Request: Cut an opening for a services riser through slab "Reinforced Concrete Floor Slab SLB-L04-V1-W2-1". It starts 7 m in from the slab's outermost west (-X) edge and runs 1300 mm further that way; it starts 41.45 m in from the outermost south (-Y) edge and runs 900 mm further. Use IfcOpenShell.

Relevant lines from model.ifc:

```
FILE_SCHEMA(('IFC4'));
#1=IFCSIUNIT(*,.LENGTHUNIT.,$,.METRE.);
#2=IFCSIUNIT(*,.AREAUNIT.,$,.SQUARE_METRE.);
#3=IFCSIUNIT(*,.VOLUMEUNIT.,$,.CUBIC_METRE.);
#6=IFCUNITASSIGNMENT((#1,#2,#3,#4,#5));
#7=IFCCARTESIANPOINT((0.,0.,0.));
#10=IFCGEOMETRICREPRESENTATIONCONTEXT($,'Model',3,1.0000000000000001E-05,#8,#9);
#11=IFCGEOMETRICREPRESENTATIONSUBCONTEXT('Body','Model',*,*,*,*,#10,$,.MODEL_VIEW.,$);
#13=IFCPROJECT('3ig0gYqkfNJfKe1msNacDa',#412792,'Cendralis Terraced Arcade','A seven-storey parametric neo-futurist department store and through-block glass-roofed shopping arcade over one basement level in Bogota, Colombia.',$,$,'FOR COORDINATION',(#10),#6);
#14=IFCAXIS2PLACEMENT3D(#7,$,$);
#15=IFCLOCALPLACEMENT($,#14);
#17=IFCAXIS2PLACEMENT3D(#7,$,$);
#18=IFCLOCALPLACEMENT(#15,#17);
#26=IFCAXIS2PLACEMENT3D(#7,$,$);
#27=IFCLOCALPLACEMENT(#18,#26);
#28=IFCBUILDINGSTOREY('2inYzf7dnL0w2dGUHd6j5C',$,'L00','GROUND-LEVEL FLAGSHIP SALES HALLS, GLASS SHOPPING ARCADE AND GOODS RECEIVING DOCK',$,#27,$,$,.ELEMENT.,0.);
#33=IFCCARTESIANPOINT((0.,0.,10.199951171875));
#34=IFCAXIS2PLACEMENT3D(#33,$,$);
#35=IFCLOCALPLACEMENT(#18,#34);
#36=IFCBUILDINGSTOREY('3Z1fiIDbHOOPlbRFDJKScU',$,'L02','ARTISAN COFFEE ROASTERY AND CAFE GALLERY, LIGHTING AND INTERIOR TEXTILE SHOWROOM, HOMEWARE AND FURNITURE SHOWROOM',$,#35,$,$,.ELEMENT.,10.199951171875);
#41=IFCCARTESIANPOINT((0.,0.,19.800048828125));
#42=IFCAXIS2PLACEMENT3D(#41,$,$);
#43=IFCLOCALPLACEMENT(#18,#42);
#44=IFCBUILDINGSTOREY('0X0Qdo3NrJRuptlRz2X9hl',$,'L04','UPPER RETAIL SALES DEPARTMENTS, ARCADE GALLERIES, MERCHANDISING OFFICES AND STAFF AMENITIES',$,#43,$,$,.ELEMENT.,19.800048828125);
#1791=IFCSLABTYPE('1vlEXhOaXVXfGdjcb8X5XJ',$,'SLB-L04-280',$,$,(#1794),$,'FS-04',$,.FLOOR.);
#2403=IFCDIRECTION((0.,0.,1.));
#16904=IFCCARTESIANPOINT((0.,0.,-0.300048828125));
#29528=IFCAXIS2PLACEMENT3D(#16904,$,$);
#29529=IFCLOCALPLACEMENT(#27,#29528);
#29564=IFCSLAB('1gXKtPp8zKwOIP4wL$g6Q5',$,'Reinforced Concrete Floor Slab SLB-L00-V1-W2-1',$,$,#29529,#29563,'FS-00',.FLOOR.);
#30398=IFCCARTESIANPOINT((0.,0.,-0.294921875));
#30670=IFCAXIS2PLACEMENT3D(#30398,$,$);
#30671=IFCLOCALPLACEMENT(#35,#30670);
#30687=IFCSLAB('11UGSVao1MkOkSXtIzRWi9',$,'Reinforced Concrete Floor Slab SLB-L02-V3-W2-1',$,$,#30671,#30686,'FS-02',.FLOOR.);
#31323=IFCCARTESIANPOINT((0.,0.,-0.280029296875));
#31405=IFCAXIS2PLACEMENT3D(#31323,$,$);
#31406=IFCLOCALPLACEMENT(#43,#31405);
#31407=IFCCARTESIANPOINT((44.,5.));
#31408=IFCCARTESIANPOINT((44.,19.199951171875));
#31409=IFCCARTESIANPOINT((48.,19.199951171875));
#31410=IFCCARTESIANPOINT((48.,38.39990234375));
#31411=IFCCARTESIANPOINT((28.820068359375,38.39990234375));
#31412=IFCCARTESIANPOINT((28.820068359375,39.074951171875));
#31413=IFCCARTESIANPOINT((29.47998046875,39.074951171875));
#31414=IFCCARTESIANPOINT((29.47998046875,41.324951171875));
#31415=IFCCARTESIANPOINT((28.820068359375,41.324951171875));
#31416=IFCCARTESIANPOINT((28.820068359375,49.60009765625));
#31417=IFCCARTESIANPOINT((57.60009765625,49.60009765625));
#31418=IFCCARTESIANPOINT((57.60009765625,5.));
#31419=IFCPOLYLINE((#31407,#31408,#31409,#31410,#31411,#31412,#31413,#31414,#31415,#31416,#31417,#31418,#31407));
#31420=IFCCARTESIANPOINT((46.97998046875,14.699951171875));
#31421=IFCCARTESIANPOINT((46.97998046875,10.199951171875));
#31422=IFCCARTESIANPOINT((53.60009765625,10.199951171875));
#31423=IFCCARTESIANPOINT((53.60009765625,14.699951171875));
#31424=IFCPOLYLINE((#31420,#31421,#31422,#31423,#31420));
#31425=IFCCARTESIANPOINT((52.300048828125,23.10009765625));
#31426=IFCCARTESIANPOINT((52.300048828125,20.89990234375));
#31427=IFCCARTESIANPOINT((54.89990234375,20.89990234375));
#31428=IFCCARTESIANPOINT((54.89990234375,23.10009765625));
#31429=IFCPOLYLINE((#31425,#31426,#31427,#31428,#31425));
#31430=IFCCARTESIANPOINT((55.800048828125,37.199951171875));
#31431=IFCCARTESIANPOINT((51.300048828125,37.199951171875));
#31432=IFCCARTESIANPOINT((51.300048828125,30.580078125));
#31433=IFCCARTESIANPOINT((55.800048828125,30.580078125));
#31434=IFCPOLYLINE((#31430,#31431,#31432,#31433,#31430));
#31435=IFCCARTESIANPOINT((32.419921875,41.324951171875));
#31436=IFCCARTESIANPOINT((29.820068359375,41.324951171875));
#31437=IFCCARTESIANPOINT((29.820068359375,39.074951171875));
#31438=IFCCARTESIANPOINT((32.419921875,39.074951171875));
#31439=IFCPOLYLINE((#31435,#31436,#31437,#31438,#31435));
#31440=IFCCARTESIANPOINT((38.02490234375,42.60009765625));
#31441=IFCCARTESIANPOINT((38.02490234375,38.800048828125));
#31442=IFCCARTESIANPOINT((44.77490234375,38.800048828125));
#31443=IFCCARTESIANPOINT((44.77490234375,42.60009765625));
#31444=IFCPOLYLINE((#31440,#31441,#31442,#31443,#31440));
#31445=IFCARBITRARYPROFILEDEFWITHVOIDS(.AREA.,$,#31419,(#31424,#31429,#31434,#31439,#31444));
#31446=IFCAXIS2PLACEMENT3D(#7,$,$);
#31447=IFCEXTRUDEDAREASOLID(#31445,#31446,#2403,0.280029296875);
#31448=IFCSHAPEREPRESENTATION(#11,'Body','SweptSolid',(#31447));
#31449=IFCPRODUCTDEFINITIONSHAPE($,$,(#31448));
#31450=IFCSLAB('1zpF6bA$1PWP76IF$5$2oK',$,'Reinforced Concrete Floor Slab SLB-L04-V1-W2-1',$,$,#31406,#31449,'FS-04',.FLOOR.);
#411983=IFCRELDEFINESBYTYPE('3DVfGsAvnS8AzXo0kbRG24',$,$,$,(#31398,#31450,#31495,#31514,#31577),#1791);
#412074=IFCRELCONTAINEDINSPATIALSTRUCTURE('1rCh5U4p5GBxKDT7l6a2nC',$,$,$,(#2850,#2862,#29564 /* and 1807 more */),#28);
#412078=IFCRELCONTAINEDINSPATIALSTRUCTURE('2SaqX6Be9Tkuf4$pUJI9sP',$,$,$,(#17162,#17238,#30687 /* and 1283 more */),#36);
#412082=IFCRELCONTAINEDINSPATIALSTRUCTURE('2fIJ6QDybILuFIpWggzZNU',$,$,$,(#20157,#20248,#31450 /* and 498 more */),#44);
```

```python
import numpy as np
import ifcopenshell
import ifcopenshell.api.feature
import ifcopenshell.api.geometry
import ifcopenshell.api.root
import ifcopenshell.geom
import ifcopenshell.util.placement
import ifcopenshell.util.representation
import ifcopenshell.util.shape
import ifcopenshell.util.unit

model = ifcopenshell.open("model.ifc")
unit_scale = ifcopenshell.util.unit.calculate_unit_scale(model)
settings = ifcopenshell.geom.settings()


def volume(element):
    """Net volume in cubic metres, openings subtracted."""
    shape = ifcopenshell.geom.create_shape(settings, element)
    return ifcopenshell.util.shape.get_volume(shape.geometry)


slab = model.by_guid("1zpF6bA$1PWP76IF$5$2oK")
before = volume(slab)

# Extent in the slab's own axes, in metres. The edges named are its -X and -Y sides.
slab_shape = ifcopenshell.geom.create_shape(settings, slab)
vertices = ifcopenshell.util.shape.get_vertices(slab_shape.geometry)
x_min, y_min, bottom = vertices.min(axis=0)
top = vertices[:, 2].max()

opening = ifcopenshell.api.root.create_entity(model, ifc_class="IfcOpeningElement", name="Services riser opening", predefined_type="OPENING")
context = ifcopenshell.util.representation.get_context(model, "Model", "Body", "MODEL_VIEW")
width, depth = 1.3, 0.9
outline = [(0.0, 0.0), (width, 0.0), (width, depth), (0.0, depth), (0.0, 0.0)]
# Overshoot both faces by 50 mm so the cut is clean.
shape = ifcopenshell.api.geometry.add_slab_representation(
    model, context=context, depth=top - bottom + 0.1, polyline=outline
)
ifcopenshell.api.geometry.assign_representation(model, product=opening, representation=shape)

matrix = ifcopenshell.util.placement.get_local_placement(slab.ObjectPlacement)
matrix[:, 3] = matrix @ np.append(np.array([x_min + 7, y_min + 41.45, bottom - 0.05]) / unit_scale, 1.0)
ifcopenshell.api.geometry.edit_object_placement(model, product=opening, matrix=matrix, is_si=False)
ifcopenshell.api.feature.add_feature(model, feature=opening, element=slab)

after = volume(slab)

print(f"slab volume {before:.3f} -> {after:.3f} m3")

model.write("model-out.ifc")
```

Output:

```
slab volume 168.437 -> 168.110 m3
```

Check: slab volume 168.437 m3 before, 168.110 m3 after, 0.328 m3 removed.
